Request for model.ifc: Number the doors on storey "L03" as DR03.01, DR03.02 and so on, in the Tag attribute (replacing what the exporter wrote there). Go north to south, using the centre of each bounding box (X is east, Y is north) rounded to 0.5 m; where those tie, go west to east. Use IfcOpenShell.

First a look at what the model holds.

```python
import ifcopenshell
import ifcopenshell.util.element
import ifcopenshell.util.placement

model = ifcopenshell.open("model.ifc")
print(model.schema)
storey = next(s for s in model.by_type("IfcBuildingStorey") if s.Name == "L03")
doors = [e for e in ifcopenshell.util.element.get_decomposition(storey) if e.is_a("IfcDoor")]
for e in sorted(doors, key=lambda e: e.id()):
    origin = ifcopenshell.util.placement.get_local_placement(e.ObjectPlacement)[:3, 3]
    print(e.id(), e.Tag, e.Name, origin.round(2) + 0.0, sep=" | ")
```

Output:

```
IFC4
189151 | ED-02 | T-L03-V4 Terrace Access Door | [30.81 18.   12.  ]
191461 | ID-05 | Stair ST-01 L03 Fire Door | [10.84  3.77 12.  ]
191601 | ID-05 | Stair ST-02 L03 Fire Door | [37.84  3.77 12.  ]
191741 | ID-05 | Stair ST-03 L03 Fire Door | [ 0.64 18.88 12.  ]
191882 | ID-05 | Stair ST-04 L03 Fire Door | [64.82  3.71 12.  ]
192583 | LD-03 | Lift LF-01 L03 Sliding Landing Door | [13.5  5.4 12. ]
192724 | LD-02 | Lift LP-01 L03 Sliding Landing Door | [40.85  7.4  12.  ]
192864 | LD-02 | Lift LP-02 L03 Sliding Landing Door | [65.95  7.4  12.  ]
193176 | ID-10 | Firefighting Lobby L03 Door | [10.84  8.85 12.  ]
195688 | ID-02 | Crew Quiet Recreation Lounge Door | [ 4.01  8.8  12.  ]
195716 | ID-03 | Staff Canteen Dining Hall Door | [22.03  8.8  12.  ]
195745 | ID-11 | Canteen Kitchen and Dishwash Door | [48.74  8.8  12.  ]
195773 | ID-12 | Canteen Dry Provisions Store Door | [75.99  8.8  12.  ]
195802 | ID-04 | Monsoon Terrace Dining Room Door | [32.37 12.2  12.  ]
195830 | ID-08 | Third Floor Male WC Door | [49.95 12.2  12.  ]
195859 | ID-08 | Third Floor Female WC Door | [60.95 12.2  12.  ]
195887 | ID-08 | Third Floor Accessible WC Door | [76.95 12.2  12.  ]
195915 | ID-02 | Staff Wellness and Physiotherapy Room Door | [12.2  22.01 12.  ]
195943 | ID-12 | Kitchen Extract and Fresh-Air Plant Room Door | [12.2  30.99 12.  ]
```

```python
import ifcopenshell
import ifcopenshell.geom
import ifcopenshell.util.element
import ifcopenshell.util.shape

model = ifcopenshell.open("model.ifc")
settings = ifcopenshell.geom.settings()
settings.set("use-world-coords", True)


def centre(element):
    shape = ifcopenshell.geom.create_shape(settings, element)
    return ifcopenshell.util.shape.get_bbox_centroid(shape.geometry)


storey = next(s for s in model.by_type("IfcBuildingStorey") if s.Name == "L03")
doors = [e for e in ifcopenshell.util.element.get_decomposition(storey) if e.is_a("IfcDoor")]

# Insertion points can sit at a corner or the storey origin, so sort by the geometry (in metres).
centres = {e: centre(e) for e in doors}
doors.sort(key=lambda e: (-round(centres[e][1] / 0.5), centres[e][0]))

for i, e in enumerate(doors, start=1):
    number = f"DR03.{i:02d}"
    e.Tag = number
    print(e.id(), number)

model.write("model-out.ifc")
```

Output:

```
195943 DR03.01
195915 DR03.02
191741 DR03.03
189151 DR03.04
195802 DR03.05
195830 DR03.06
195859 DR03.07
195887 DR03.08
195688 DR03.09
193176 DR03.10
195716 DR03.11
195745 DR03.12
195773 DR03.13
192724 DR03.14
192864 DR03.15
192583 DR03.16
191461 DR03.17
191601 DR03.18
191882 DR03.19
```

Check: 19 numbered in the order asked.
